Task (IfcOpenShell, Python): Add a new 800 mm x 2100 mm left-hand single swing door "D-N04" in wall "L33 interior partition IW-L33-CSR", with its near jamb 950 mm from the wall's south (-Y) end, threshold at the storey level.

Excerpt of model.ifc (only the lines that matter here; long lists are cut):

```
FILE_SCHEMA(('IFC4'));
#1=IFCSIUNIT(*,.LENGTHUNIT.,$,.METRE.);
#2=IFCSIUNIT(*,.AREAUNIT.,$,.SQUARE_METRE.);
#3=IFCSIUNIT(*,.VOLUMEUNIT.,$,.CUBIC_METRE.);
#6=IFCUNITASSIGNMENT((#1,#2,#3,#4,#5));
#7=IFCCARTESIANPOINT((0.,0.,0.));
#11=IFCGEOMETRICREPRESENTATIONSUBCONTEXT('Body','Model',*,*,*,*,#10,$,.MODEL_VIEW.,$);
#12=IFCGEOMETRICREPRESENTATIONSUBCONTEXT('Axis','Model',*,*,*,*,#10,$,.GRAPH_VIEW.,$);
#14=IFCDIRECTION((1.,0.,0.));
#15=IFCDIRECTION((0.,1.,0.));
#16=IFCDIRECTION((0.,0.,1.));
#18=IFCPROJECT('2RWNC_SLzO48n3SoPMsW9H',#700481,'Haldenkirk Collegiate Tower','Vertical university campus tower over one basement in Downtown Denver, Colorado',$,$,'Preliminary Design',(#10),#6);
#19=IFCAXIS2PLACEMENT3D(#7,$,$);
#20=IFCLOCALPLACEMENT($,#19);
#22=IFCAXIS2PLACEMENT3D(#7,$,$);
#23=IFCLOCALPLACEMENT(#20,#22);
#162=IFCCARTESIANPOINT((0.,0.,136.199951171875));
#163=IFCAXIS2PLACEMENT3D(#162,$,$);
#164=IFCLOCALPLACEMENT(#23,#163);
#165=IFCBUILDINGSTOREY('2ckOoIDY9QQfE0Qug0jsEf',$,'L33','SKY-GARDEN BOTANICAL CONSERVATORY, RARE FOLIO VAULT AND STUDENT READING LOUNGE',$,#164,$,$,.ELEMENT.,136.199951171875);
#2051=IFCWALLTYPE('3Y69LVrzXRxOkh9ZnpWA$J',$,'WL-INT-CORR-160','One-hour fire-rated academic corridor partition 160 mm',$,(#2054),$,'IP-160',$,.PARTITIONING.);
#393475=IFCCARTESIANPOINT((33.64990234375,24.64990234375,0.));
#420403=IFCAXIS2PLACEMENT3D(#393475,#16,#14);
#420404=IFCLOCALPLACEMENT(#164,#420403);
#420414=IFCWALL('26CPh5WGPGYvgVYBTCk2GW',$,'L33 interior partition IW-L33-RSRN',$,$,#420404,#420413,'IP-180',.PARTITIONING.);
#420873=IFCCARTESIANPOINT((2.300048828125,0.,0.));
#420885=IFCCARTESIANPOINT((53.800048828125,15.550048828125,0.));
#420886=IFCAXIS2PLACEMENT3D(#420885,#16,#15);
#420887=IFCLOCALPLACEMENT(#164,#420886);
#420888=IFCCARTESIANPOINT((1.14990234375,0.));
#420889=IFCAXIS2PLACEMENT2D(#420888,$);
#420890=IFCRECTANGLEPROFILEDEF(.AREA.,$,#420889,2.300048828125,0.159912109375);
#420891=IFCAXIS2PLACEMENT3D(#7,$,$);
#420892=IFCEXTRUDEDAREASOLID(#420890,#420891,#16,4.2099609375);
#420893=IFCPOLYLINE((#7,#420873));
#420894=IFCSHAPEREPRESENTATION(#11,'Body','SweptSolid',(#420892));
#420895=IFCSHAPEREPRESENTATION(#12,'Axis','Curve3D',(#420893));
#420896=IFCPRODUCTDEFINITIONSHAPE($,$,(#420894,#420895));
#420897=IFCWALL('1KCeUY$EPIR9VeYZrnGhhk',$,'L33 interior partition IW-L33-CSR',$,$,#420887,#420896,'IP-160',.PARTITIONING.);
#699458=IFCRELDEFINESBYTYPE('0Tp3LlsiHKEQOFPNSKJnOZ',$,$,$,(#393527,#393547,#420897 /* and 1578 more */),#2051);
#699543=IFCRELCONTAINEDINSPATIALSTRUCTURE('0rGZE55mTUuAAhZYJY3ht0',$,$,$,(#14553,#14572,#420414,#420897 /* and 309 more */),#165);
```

```python
import numpy as np
import ifcopenshell
import ifcopenshell.api.feature
import ifcopenshell.api.geometry
import ifcopenshell.api.root
import ifcopenshell.api.spatial
import ifcopenshell.geom
import ifcopenshell.util.element
import ifcopenshell.util.placement
import ifcopenshell.util.representation
import ifcopenshell.util.shape
import ifcopenshell.util.unit

model = ifcopenshell.open("model.ifc")
unit_scale = ifcopenshell.util.unit.calculate_unit_scale(model)
settings = ifcopenshell.geom.settings()


def volume(element):
    """Net volume in cubic metres, openings subtracted."""
    shape = ifcopenshell.geom.create_shape(settings, element)
    return ifcopenshell.util.shape.get_volume(shape.geometry)


wall = model.by_guid("1KCeUY$EPIR9VeYZrnGhhk")
storey = ifcopenshell.util.element.get_container(wall, ifc_class="IfcBuildingStorey")
context = ifcopenshell.util.representation.get_context(model, "Model", "Body", "MODEL_VIEW")
before = volume(wall)

width, height, from_end, sill = 0.8, 2.1, 0.95, 0.0  # metres

# The wall runs along its own X axis, and the end named is its -X end.
wall_shape = ifcopenshell.geom.create_shape(settings, wall)
x, y, z = ifcopenshell.util.shape.get_vertices(wall_shape.geometry).T
start = x.min() + from_end
face, thickness = float(y.min()), float(y.max() - y.min())
wall_matrix = ifcopenshell.util.placement.get_local_placement(wall.ObjectPlacement)
level = ifcopenshell.util.placement.get_local_placement(storey.ObjectPlacement)[2, 3]


def in_wall(x, y):
    """Placement at x, y metres in the wall's axes, at sill height."""
    matrix = wall_matrix.copy()
    matrix[:, 3] = wall_matrix @ np.array([x / unit_scale, y / unit_scale, 0.0, 1.0])
    matrix[2, 3] = level + sill / unit_scale
    return matrix


# Opening: a box that overshoots both wall faces by 50 mm.
opening = ifcopenshell.api.root.create_entity(model, ifc_class="IfcOpeningElement", predefined_type="OPENING")
box = ifcopenshell.api.geometry.add_wall_representation(
    model, context=context, length=width, height=height, thickness=thickness + 0.1
)
ifcopenshell.api.geometry.assign_representation(model, product=opening, representation=box)
ifcopenshell.api.geometry.edit_object_placement(model, product=opening, matrix=in_wall(start, face - 0.05), is_si=False)
ifcopenshell.api.feature.add_feature(model, feature=opening, element=wall)

door = ifcopenshell.api.root.create_entity(model, ifc_class="IfcDoor", name="D-N04", predefined_type="DOOR")
door.OverallWidth, door.OverallHeight = width / unit_scale, height / unit_scale
door.OperationType = "SINGLE_SWING_LEFT"
body = ifcopenshell.api.geometry.add_door_representation(
    model,
    context=context,
    overall_width=door.OverallWidth,
    overall_height=door.OverallHeight,
    operation_type="SINGLE_SWING_LEFT",
    lining_properties={"LiningDepth": thickness / unit_scale, "ThresholdDepth": thickness / unit_scale},
)
ifcopenshell.api.geometry.assign_representation(model, product=door, representation=body)
ifcopenshell.api.spatial.assign_container(model, products=[door], relating_structure=storey)
ifcopenshell.api.feature.add_filling(model, opening=opening, element=door)

# The lining spans the wall, so the door starts at the wall face.
ifcopenshell.api.geometry.edit_object_placement(model, product=door, matrix=in_wall(start, face), is_si=False)

after = volume(wall)

print(f"wall volume {before:.3f} -> {after:.3f} m3")

model.write("model-out.ifc")
```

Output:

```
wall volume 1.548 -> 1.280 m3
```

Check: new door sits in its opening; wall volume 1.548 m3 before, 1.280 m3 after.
